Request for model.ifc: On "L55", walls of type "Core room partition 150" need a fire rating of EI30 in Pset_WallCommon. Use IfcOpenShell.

First a look at what the model holds.

```python
import ifcopenshell
import ifcopenshell.util.element

model = ifcopenshell.open("model.ifc")
print(model.schema)
storey = next(s for s in model.by_type("IfcBuildingStorey") if s.Name == "L55")
walls = [e for e in ifcopenshell.util.element.get_decomposition(storey) if e.is_a("IfcWall")]
seen = {}
for e in walls:
    element_type = ifcopenshell.util.element.get_type(e)
    key = (element_type.Name if element_type != e and element_type else None, ifcopenshell.util.element.get_pset(e, "Pset_WallCommon", "FireRating"))
    seen[key] = seen.get(key, 0) + 1
for (name, value), count in sorted(seen.items(), key=str):
    print(count, "x", name, "|", value)
```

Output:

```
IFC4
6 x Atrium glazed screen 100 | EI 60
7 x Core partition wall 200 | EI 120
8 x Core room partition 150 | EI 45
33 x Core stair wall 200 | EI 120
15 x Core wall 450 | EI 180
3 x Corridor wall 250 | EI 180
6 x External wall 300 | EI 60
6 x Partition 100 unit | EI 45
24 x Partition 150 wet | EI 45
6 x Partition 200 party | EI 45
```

```python
import ifcopenshell
import ifcopenshell.api.pset
import ifcopenshell.util.element

model = ifcopenshell.open("model.ifc")

storey = next(s for s in model.by_type("IfcBuildingStorey") if s.Name == "L55")
walls = [e for e in ifcopenshell.util.element.get_decomposition(storey) if e.is_a("IfcWall")]

count = 0
for e in walls:
    element_type = ifcopenshell.util.element.get_type(e)
    if element_type in (None, e) or element_type.Name != "Core room partition 150":
        continue
    found = ifcopenshell.util.element.get_pset(e, "Pset_WallCommon", should_inherit=False)
    if found:
        pset = model.by_id(found["id"])
        if len(ifcopenshell.util.element.get_elements_by_pset(pset)) > 1:
            pset = ifcopenshell.api.pset.unshare_pset(model, products=[e], pset=pset)[0]
    else:
        pset = ifcopenshell.api.pset.add_pset(model, product=e, name="Pset_WallCommon")
    ifcopenshell.api.pset.edit_pset(model, pset=pset, properties={"FireRating": "EI30"})
    count += 1

print(count, "walls updated")

model.write("model_rev.ifc")
```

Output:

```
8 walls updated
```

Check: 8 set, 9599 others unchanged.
